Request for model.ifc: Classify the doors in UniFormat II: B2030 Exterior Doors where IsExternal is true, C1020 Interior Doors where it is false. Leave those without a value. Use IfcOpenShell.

First a look at what the model holds.

```python
import ifcopenshell
import ifcopenshell.util.element

model = ifcopenshell.open("model.ifc")
print(model.schema)
print("classifications:", [c.Name for c in model.by_type("IfcClassification")])
values = [ifcopenshell.util.element.get_pset(e, "Pset_DoorCommon", "IsExternal") for e in model.by_type("IfcDoor")]
for value in (True, False, None):
    print("IsExternal", value, values.count(value))
```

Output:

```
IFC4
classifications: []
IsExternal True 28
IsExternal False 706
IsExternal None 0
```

```python
import ifcopenshell
import ifcopenshell.api.classification
import ifcopenshell.util.element

model = ifcopenshell.open("model.ifc")

system = ifcopenshell.api.classification.add_classification(model, classification="UniFormat II")

doors = model.by_type("IfcDoor")
external = {e: ifcopenshell.util.element.get_pset(e, "Pset_DoorCommon", "IsExternal") for e in doors}
for flag, code, name in ((True, "B2030", "Exterior Doors"), (False, "C1020", "Interior Doors")):
    products = [e for e in doors if external[e] is flag]
    ifcopenshell.api.classification.add_reference(
        model, products=products, classification=system, identification=code, name=name
    )
    print(code, len(products))

model.write("model_v2.ifc")
```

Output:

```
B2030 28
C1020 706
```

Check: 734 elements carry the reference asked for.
